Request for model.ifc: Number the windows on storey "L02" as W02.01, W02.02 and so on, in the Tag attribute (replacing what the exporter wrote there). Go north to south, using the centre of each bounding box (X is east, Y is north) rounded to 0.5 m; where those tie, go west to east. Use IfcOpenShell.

First a look at what the model holds.

```python
import ifcopenshell
import ifcopenshell.util.element
import ifcopenshell.util.placement

model = ifcopenshell.open("model.ifc")
print(model.schema)
storey = next(s for s in model.by_type("IfcBuildingStorey") if s.Name == "L02")
windows = [e for e in ifcopenshell.util.element.get_decomposition(storey) if e.is_a("IfcWindow")]
for e in sorted(windows, key=lambda e: e.id()):
    origin = ifcopenshell.util.placement.get_local_placement(e.ObjectPlacement)[:3, 3]
    print(e.id(), e.Tag, e.Name, origin.round(2) + 0.0, sep=" | ")
```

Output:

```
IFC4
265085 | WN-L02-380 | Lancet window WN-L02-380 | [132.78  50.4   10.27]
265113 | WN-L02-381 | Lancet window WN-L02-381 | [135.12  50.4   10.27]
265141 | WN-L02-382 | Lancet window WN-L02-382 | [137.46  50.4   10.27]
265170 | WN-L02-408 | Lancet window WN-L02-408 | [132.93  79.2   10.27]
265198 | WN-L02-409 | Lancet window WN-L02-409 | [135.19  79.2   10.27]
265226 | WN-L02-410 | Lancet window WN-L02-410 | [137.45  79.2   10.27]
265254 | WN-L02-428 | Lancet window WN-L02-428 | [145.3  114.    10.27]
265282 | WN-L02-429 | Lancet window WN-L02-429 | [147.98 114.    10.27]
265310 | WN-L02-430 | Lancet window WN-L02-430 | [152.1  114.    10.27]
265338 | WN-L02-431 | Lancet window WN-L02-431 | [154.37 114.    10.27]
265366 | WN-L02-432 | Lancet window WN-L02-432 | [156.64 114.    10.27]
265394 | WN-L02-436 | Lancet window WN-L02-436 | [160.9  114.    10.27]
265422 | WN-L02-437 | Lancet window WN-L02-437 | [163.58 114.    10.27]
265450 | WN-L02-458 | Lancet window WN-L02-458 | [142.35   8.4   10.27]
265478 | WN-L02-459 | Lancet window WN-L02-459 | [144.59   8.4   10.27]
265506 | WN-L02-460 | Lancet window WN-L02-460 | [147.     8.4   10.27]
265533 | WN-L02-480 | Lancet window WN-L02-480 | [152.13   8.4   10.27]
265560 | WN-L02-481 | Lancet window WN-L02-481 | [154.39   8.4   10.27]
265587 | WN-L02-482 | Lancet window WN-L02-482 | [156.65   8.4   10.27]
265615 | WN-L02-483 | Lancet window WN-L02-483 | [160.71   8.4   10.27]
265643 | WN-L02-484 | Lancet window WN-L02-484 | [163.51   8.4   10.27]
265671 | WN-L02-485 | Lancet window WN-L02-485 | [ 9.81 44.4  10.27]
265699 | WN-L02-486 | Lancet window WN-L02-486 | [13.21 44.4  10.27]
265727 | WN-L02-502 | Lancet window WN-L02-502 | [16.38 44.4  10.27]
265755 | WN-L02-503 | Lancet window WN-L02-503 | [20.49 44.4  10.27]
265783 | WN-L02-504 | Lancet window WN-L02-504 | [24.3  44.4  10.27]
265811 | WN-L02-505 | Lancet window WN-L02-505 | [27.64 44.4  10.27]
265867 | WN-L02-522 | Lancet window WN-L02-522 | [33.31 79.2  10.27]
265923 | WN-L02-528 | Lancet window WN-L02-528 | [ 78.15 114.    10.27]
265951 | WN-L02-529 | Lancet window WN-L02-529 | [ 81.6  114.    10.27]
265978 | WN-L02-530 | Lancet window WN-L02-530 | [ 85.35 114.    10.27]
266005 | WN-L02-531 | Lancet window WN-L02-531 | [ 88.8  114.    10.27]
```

```python
import ifcopenshell
import ifcopenshell.geom
import ifcopenshell.util.element
import ifcopenshell.util.shape

model = ifcopenshell.open("model.ifc")
settings = ifcopenshell.geom.settings()
settings.set("use-world-coords", True)


def centre(element):
    shape = ifcopenshell.geom.create_shape(settings, element)
    return ifcopenshell.util.shape.get_bbox_centroid(shape.geometry)


storey = next(s for s in model.by_type("IfcBuildingStorey") if s.Name == "L02")
windows = [e for e in ifcopenshell.util.element.get_decomposition(storey) if e.is_a("IfcWindow")]

# Insertion points can sit at a corner or the storey origin, so sort by the geometry (in metres).
centres = {e: centre(e) for e in windows}
windows.sort(key=lambda e: (-round(centres[e][1] / 0.5), centres[e][0]))

for i, e in enumerate(windows, start=1):
    number = f"W02.{i:02d}"
    e.Tag = number
    print(e.id(), number)

model.write("model_v2.ifc")
```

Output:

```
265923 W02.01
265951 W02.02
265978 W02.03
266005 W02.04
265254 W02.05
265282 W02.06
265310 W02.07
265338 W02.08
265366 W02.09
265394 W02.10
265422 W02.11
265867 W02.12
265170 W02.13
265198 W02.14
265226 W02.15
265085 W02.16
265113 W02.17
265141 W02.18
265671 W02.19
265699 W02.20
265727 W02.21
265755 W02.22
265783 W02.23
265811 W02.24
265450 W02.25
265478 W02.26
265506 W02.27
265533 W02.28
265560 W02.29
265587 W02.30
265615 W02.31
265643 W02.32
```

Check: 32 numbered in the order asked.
